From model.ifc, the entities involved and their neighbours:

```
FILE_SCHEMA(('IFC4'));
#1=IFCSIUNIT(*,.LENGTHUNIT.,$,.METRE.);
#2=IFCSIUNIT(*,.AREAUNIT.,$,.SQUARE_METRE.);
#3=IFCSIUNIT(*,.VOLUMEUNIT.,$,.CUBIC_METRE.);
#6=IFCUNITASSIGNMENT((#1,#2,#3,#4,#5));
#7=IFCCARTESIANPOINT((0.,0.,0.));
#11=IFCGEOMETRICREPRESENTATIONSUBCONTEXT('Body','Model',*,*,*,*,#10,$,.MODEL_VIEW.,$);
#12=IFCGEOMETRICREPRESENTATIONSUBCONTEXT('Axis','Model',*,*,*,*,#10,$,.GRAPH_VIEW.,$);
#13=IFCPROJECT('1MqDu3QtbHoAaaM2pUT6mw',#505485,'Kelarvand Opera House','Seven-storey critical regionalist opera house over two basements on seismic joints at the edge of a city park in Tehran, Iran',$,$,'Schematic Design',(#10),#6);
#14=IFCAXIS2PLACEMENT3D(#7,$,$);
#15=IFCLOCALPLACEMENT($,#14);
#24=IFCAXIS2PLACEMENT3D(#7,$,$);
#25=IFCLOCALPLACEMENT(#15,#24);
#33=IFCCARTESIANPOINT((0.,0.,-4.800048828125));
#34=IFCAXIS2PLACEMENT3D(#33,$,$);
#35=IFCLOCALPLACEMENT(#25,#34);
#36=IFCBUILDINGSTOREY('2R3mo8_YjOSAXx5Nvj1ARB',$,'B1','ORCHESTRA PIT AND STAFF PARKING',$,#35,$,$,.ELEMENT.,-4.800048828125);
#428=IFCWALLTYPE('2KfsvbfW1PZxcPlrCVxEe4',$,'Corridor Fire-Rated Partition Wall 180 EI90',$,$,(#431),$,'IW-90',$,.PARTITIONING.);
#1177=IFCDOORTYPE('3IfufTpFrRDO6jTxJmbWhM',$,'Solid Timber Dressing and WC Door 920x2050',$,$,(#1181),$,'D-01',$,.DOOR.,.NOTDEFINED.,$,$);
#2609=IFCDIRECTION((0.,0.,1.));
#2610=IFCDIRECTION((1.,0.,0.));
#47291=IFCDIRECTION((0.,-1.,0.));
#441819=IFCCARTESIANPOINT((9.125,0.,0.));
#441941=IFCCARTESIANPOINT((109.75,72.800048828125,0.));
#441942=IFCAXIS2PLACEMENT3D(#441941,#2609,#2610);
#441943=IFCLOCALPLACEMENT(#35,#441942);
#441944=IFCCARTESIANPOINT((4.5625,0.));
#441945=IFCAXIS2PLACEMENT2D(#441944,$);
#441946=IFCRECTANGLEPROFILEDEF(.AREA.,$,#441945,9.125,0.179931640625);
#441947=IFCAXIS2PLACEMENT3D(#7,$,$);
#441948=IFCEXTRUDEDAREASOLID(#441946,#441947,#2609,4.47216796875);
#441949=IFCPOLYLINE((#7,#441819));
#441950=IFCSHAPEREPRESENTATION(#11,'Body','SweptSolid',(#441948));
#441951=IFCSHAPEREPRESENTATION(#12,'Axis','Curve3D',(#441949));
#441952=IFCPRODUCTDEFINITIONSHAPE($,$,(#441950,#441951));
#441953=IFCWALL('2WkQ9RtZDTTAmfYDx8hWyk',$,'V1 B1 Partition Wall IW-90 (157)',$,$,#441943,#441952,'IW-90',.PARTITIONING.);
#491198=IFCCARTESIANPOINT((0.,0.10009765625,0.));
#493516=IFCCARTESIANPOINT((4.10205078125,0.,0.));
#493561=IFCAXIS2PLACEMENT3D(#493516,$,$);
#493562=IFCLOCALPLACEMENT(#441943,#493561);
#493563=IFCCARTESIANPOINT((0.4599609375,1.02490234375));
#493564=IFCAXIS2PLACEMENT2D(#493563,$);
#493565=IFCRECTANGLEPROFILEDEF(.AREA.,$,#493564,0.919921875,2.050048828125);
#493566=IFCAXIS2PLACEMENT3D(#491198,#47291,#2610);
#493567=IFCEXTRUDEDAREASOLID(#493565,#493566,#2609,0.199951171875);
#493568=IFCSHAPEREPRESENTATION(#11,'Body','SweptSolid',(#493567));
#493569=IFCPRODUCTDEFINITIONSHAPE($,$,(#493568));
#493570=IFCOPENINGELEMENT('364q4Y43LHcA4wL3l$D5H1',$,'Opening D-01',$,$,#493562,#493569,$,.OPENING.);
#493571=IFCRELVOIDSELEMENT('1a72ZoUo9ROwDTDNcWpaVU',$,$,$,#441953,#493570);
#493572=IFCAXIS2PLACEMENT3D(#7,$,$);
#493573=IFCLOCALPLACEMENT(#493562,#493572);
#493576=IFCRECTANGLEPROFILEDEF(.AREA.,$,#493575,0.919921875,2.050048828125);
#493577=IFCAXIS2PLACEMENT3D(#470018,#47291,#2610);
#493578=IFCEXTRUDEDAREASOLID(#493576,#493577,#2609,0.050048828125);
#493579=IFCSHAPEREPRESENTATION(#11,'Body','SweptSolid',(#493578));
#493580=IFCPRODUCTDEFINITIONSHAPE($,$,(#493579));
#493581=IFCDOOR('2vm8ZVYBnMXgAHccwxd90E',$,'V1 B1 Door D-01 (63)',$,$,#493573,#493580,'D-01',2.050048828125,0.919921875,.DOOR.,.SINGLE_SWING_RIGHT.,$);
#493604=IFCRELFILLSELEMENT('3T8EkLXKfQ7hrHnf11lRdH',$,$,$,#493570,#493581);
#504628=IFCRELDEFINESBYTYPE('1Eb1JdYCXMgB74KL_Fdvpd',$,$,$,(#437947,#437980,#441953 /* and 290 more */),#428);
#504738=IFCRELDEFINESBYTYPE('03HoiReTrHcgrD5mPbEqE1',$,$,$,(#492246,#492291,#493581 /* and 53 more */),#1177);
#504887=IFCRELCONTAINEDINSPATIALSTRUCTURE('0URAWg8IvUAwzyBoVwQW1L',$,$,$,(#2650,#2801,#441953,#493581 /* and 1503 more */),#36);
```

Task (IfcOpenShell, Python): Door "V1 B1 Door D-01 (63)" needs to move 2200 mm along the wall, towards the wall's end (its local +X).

```python
import ifcopenshell
import ifcopenshell.api.geometry
import ifcopenshell.util.placement
import ifcopenshell.util.unit

model = ifcopenshell.open("model.ifc")
unit_scale = ifcopenshell.util.unit.calculate_unit_scale(model)

door = model.by_guid("2vm8ZVYBnMXgAHccwxd90E")
opening = door.FillsVoids[0].RelatingOpeningElement
wall = opening.VoidsElements[0].RelatingBuildingElement

wall_matrix = ifcopenshell.util.placement.get_local_placement(wall.ObjectPlacement)
shift = wall_matrix[:3, 0] * 2.2 / unit_scale
before = ifcopenshell.util.placement.get_local_placement(door.ObjectPlacement)[:3, 3].copy()

# The door is placed relative to its opening, so it follows when the opening moves.
matrix = ifcopenshell.util.placement.get_local_placement(opening.ObjectPlacement)
matrix[:3, 3] += shift
ifcopenshell.api.geometry.edit_object_placement(
    model, product=opening, matrix=matrix, is_si=False, should_transform_children=True
)

after = ifcopenshell.util.placement.get_local_placement(door.ObjectPlacement)[:3, 3]
print("door moved by", (after - before).round(3) + 0.0)

model.write("model_v2.ifc")
```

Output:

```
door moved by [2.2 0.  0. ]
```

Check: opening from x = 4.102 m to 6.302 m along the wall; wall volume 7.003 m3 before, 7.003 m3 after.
